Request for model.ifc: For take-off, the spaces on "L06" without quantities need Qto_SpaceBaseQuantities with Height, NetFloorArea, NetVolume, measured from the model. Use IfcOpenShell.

First a look at what the model holds.

```python
import ifcopenshell
import ifcopenshell.util.element
import ifcopenshell.util.unit

model = ifcopenshell.open("model.ifc")
print(model.schema)
for unit_type in ("LENGTHUNIT", "AREAUNIT", "VOLUMEUNIT"):
    print(unit_type, ifcopenshell.util.unit.calculate_unit_scale(model, unit_type))
storey = next(s for s in model.by_type("IfcBuildingStorey") if s.Name == "L06")
spaces = [e for e in ifcopenshell.util.element.get_decomposition(storey) if e.is_a("IfcSpace")]
for e in sorted(spaces, key=lambda e: e.id()):
    print(e.id(), e.is_a(), e.Name, list(ifcopenshell.util.element.get_psets(e, qtos_only=True)), sep=" | ")
```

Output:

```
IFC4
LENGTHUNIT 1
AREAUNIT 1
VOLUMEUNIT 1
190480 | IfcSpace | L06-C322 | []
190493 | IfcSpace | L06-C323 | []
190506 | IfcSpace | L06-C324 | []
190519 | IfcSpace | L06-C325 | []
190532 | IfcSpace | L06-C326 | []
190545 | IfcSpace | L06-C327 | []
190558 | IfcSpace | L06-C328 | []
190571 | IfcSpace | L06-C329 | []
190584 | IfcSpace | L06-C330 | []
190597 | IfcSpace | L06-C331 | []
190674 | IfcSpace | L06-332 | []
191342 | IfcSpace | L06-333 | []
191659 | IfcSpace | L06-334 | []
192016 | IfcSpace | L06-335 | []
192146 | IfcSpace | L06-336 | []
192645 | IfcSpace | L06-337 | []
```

```python
import ifcopenshell
import ifcopenshell.api.pset
import ifcopenshell.geom
import ifcopenshell.util.element
import ifcopenshell.util.shape
import ifcopenshell.util.unit

model = ifcopenshell.open("model.ifc")
unit_scale = ifcopenshell.util.unit.calculate_unit_scale(model)
area_scale = ifcopenshell.util.unit.calculate_unit_scale(model, "AREAUNIT")
volume_scale = ifcopenshell.util.unit.calculate_unit_scale(model, "VOLUMEUNIT")
settings = ifcopenshell.geom.settings()

storey = next(s for s in model.by_type("IfcBuildingStorey") if s.Name == "L06")
spaces = [e for e in ifcopenshell.util.element.get_decomposition(storey) if e.is_a("IfcSpace")]

for e in sorted(spaces, key=lambda e: e.id()):
    if ifcopenshell.util.element.get_psets(e, qtos_only=True, should_inherit=False):
        continue
    # Geometry comes back in metres, in the element's own axes.
    shape = ifcopenshell.geom.create_shape(settings, e)
    values = {
        "Height": ifcopenshell.util.shape.get_z(shape.geometry) / unit_scale,
        "NetFloorArea": ifcopenshell.util.shape.get_footprint_area(shape.geometry) / area_scale,
        "NetVolume": ifcopenshell.util.shape.get_volume(shape.geometry) / volume_scale,
    }
    qto = ifcopenshell.api.pset.add_qto(model, product=e, name="Qto_SpaceBaseQuantities")
    ifcopenshell.api.pset.edit_qto(model, qto=qto, properties=values)
    print(e.id(), {k: round(v, 3) for k, v in values.items()})

model.write("model_rev.ifc")
```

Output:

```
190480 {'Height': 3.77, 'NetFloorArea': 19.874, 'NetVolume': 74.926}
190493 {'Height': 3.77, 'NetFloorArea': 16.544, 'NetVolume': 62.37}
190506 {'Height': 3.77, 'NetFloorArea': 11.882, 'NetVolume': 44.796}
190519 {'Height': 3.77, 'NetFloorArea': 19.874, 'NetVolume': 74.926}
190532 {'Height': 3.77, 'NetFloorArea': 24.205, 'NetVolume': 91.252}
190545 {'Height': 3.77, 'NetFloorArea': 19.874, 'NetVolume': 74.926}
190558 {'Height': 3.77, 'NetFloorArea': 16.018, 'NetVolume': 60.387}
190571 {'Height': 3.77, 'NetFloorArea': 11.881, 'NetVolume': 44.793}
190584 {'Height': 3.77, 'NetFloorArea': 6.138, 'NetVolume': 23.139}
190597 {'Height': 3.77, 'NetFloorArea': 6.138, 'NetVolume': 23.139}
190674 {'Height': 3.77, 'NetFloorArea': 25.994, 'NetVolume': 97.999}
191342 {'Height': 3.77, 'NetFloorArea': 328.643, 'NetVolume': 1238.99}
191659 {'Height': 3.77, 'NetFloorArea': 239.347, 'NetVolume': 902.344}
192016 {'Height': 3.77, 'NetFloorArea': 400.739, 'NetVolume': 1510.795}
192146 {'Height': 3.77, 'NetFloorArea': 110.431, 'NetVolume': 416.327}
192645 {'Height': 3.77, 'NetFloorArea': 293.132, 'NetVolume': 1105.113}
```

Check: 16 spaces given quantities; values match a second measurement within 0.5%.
